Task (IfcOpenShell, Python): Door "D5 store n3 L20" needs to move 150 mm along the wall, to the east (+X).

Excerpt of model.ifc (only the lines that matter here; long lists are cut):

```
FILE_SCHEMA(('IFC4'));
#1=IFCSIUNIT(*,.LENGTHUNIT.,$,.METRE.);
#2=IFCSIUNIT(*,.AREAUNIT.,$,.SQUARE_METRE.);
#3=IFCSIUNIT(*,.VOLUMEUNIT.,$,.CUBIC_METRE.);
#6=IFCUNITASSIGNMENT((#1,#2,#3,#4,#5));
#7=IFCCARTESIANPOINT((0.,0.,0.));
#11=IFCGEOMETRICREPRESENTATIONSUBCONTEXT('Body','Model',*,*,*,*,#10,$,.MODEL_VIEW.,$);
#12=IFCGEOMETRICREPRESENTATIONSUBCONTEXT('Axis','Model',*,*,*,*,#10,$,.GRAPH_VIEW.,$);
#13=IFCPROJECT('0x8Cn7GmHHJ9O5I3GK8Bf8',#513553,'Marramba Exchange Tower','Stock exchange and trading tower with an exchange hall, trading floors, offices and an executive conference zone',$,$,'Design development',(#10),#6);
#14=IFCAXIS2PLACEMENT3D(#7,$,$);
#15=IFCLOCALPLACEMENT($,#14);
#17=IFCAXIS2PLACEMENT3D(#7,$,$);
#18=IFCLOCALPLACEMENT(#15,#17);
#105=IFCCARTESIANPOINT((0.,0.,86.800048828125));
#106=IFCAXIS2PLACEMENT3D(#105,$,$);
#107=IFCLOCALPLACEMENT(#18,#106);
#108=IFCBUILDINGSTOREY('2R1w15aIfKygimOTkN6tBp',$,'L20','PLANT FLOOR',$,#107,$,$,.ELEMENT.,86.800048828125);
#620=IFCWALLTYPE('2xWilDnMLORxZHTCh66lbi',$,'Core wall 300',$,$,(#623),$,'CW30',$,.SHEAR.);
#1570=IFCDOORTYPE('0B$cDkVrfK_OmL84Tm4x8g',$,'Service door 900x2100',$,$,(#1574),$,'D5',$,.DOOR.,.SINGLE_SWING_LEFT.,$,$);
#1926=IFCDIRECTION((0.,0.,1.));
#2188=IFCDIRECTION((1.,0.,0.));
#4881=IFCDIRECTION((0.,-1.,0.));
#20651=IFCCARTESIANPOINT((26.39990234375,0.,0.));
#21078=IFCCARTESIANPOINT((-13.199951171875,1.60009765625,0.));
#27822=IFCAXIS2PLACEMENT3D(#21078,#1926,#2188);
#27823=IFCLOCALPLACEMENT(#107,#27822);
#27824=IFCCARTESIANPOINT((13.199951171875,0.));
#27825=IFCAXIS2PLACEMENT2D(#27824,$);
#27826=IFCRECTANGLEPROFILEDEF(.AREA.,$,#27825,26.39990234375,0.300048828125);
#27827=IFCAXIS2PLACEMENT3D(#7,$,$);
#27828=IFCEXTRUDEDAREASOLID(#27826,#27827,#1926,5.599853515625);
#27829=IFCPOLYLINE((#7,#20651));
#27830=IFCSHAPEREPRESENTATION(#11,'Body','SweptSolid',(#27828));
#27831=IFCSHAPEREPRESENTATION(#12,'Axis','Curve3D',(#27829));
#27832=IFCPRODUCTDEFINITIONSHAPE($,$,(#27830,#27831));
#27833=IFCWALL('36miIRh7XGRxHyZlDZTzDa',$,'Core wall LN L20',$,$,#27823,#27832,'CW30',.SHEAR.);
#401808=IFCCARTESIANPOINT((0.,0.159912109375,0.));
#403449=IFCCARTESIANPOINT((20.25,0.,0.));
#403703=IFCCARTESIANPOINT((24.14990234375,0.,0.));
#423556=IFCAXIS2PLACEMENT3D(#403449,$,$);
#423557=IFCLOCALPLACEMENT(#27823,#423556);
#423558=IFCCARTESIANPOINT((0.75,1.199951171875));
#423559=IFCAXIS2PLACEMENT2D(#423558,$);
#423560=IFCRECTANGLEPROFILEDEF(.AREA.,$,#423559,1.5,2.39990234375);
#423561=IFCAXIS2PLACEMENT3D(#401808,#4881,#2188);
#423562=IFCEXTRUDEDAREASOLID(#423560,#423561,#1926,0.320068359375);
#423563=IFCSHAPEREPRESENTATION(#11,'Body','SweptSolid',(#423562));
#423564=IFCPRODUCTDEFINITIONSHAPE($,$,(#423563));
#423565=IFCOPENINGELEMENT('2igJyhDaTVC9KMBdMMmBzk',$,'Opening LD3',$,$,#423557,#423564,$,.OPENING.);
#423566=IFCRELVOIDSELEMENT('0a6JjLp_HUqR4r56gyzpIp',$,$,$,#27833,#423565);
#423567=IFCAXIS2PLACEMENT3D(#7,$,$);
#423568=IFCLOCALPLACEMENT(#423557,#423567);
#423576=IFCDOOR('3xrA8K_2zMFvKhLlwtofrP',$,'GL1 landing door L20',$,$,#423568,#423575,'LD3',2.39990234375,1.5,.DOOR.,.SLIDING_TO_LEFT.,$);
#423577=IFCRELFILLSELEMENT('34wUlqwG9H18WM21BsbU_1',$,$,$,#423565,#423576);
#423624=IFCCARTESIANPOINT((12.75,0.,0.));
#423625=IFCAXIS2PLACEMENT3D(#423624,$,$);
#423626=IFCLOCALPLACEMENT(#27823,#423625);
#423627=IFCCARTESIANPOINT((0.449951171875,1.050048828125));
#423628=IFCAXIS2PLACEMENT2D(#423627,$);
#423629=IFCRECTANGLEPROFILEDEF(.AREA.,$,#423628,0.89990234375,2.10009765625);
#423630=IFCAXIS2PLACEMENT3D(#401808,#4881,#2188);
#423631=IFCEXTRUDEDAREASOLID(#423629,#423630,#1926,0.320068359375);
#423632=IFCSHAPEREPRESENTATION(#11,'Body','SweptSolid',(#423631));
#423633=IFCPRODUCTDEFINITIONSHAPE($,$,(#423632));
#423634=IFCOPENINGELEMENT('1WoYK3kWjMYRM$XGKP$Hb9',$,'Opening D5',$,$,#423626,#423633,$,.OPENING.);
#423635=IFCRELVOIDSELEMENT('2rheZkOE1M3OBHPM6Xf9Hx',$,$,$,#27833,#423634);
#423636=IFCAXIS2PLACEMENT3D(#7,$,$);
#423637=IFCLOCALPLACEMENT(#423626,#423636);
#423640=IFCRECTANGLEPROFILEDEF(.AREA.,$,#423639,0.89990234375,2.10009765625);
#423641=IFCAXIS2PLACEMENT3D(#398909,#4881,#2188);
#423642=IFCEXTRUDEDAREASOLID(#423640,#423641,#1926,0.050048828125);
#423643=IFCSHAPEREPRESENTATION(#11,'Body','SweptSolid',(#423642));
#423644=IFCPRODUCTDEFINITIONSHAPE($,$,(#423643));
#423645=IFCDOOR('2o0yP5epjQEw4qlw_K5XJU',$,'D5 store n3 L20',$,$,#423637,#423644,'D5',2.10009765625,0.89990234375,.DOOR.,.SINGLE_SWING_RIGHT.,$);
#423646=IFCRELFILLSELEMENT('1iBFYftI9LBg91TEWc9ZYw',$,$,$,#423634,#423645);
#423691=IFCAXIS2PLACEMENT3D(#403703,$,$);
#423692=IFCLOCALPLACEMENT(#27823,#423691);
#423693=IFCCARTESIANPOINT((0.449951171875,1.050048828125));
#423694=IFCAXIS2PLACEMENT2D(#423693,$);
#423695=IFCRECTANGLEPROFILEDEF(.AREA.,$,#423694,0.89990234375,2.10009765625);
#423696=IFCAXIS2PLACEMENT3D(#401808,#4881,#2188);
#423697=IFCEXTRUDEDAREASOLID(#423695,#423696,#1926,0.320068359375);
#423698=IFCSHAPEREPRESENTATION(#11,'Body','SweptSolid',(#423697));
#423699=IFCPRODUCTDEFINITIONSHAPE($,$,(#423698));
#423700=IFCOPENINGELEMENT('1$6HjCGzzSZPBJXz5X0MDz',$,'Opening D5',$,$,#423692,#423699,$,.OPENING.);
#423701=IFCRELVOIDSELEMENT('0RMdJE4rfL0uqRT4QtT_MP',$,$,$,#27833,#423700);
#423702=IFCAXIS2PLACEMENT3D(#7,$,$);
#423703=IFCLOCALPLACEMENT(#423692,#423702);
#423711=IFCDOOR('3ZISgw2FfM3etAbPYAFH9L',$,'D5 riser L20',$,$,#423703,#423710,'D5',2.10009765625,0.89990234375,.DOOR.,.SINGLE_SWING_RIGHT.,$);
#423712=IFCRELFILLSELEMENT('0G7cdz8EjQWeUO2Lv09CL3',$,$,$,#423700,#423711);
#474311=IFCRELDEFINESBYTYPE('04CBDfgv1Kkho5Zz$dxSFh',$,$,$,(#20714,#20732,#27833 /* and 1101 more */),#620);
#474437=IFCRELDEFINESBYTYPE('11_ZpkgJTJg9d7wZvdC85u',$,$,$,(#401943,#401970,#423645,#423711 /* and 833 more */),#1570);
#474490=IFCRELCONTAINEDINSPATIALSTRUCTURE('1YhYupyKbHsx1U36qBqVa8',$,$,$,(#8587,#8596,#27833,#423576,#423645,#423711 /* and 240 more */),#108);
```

```python
import ifcopenshell
import ifcopenshell.api.geometry
import ifcopenshell.util.placement

model = ifcopenshell.open("model.ifc")

door = model.by_guid("2o0yP5epjQEw4qlw_K5XJU")
opening = door.FillsVoids[0].RelatingOpeningElement
wall = opening.VoidsElements[0].RelatingBuildingElement

wall_matrix = ifcopenshell.util.placement.get_local_placement(wall.ObjectPlacement)
shift = wall_matrix[:3, 0] * 0.15
before = ifcopenshell.util.placement.get_local_placement(door.ObjectPlacement)[:3, 3].copy()

# The door is placed relative to its opening, so it follows when the opening moves.
matrix = ifcopenshell.util.placement.get_local_placement(opening.ObjectPlacement)
matrix[:3, 3] += shift
ifcopenshell.api.geometry.edit_object_placement(
    model, product=opening, matrix=matrix, is_si=False, should_transform_children=True
)

after = ifcopenshell.util.placement.get_local_placement(door.ObjectPlacement)[:3, 3]
print("door moved by", (after - before).round(3) + 0.0)

model.write("model_rev.ifc")
```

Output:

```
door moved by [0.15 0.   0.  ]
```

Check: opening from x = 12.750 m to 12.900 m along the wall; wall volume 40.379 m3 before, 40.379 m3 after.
